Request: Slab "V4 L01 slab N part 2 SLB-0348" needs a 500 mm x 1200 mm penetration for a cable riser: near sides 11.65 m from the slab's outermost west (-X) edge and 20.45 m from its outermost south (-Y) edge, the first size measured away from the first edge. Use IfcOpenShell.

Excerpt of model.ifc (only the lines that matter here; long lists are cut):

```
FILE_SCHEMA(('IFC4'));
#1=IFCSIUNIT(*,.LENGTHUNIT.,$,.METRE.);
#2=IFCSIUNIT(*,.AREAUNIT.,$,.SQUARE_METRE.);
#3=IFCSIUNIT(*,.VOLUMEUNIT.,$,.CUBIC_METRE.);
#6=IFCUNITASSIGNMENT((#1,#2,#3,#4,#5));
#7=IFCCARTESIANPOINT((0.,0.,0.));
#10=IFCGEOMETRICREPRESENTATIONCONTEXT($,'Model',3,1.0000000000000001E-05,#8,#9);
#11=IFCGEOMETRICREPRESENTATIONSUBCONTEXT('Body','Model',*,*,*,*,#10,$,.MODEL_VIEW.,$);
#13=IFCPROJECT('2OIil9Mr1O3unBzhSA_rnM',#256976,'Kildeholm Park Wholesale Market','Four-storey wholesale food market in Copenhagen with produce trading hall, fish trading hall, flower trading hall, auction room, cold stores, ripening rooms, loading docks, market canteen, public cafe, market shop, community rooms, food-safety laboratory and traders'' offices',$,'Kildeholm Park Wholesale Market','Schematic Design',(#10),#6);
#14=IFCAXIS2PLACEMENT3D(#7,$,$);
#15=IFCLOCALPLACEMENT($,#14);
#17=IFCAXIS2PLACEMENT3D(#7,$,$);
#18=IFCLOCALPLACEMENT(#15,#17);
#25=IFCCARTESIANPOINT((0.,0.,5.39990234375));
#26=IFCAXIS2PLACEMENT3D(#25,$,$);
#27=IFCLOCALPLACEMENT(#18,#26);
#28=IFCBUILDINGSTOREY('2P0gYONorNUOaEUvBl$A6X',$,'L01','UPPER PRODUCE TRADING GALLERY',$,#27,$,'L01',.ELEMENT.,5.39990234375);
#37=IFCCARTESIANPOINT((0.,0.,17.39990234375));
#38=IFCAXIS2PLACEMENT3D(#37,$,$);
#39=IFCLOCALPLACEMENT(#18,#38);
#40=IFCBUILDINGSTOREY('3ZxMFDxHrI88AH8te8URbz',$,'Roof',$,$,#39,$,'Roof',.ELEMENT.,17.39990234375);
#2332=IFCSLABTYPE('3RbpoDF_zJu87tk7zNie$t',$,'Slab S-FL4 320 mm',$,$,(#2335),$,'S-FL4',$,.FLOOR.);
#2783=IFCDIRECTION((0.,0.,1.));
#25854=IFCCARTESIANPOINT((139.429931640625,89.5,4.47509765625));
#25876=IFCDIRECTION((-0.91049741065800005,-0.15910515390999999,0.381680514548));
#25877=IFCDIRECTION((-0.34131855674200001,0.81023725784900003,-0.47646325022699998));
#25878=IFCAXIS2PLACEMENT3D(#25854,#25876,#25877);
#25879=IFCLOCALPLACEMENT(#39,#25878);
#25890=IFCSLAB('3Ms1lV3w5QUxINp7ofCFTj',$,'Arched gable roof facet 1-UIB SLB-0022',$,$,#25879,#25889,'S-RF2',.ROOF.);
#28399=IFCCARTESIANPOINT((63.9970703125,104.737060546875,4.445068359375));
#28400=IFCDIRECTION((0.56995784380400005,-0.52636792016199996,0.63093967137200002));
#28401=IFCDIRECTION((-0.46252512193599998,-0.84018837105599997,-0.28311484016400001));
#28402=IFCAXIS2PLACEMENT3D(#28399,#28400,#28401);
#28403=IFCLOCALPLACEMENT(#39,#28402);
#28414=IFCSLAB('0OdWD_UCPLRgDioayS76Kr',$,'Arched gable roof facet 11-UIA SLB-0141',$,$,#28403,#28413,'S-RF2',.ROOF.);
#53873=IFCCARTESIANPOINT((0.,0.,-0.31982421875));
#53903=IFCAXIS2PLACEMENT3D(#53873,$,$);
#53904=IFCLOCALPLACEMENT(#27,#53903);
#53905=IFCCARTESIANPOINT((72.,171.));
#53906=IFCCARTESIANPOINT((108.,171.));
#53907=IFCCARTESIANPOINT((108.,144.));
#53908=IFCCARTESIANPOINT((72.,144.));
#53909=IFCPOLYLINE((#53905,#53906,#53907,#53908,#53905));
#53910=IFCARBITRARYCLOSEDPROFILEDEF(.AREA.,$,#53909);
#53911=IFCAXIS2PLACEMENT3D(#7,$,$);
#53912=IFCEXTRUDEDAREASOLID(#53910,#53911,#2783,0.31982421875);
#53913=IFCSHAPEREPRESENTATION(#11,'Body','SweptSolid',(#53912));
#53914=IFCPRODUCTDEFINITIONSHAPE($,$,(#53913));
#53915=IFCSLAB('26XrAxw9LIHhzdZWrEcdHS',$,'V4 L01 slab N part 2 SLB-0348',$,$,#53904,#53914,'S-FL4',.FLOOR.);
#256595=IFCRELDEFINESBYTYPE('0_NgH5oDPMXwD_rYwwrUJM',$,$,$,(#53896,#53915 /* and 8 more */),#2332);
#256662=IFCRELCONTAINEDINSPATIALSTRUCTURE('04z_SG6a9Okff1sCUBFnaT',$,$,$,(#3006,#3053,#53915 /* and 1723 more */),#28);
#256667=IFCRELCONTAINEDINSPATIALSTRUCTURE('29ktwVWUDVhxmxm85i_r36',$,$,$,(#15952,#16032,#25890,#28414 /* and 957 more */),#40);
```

```python
import numpy as np
import ifcopenshell
import ifcopenshell.api.feature
import ifcopenshell.api.geometry
import ifcopenshell.api.root
import ifcopenshell.geom
import ifcopenshell.util.placement
import ifcopenshell.util.representation
import ifcopenshell.util.shape
import ifcopenshell.util.unit

model = ifcopenshell.open("model.ifc")
unit_scale = ifcopenshell.util.unit.calculate_unit_scale(model)
settings = ifcopenshell.geom.settings()


def volume(element):
    """Net volume in cubic metres, openings subtracted."""
    shape = ifcopenshell.geom.create_shape(settings, element)
    return ifcopenshell.util.shape.get_volume(shape.geometry)


slab = model.by_guid("26XrAxw9LIHhzdZWrEcdHS")
before = volume(slab)

# Extent in the slab's own axes, in metres. The edges named are its -X and -Y sides.
slab_shape = ifcopenshell.geom.create_shape(settings, slab)
vertices = ifcopenshell.util.shape.get_vertices(slab_shape.geometry)
x_min, y_min, bottom = vertices.min(axis=0)
top = vertices[:, 2].max()

opening = ifcopenshell.api.root.create_entity(model, ifc_class="IfcOpeningElement", name="Cable riser opening", predefined_type="OPENING")
context = ifcopenshell.util.representation.get_context(model, "Model", "Body", "MODEL_VIEW")
width, depth = 0.5, 1.2
outline = [(0.0, 0.0), (width, 0.0), (width, depth), (0.0, depth), (0.0, 0.0)]
# Overshoot both faces by 50 mm so the cut is clean.
shape = ifcopenshell.api.geometry.add_slab_representation(
    model, context=context, depth=top - bottom + 0.1, polyline=outline
)
ifcopenshell.api.geometry.assign_representation(model, product=opening, representation=shape)

matrix = ifcopenshell.util.placement.get_local_placement(slab.ObjectPlacement)
matrix[:, 3] = matrix @ np.append(np.array([x_min + 11.65, y_min + 20.45, bottom - 0.05]) / unit_scale, 1.0)
ifcopenshell.api.geometry.edit_object_placement(model, product=opening, matrix=matrix, is_si=False)
ifcopenshell.api.feature.add_feature(model, feature=opening, element=slab)

after = volume(slab)

print(f"slab volume {before:.3f} -> {after:.3f} m3")

model.write("model_edited.ifc")
```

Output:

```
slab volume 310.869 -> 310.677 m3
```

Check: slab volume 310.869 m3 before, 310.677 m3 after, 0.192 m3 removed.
